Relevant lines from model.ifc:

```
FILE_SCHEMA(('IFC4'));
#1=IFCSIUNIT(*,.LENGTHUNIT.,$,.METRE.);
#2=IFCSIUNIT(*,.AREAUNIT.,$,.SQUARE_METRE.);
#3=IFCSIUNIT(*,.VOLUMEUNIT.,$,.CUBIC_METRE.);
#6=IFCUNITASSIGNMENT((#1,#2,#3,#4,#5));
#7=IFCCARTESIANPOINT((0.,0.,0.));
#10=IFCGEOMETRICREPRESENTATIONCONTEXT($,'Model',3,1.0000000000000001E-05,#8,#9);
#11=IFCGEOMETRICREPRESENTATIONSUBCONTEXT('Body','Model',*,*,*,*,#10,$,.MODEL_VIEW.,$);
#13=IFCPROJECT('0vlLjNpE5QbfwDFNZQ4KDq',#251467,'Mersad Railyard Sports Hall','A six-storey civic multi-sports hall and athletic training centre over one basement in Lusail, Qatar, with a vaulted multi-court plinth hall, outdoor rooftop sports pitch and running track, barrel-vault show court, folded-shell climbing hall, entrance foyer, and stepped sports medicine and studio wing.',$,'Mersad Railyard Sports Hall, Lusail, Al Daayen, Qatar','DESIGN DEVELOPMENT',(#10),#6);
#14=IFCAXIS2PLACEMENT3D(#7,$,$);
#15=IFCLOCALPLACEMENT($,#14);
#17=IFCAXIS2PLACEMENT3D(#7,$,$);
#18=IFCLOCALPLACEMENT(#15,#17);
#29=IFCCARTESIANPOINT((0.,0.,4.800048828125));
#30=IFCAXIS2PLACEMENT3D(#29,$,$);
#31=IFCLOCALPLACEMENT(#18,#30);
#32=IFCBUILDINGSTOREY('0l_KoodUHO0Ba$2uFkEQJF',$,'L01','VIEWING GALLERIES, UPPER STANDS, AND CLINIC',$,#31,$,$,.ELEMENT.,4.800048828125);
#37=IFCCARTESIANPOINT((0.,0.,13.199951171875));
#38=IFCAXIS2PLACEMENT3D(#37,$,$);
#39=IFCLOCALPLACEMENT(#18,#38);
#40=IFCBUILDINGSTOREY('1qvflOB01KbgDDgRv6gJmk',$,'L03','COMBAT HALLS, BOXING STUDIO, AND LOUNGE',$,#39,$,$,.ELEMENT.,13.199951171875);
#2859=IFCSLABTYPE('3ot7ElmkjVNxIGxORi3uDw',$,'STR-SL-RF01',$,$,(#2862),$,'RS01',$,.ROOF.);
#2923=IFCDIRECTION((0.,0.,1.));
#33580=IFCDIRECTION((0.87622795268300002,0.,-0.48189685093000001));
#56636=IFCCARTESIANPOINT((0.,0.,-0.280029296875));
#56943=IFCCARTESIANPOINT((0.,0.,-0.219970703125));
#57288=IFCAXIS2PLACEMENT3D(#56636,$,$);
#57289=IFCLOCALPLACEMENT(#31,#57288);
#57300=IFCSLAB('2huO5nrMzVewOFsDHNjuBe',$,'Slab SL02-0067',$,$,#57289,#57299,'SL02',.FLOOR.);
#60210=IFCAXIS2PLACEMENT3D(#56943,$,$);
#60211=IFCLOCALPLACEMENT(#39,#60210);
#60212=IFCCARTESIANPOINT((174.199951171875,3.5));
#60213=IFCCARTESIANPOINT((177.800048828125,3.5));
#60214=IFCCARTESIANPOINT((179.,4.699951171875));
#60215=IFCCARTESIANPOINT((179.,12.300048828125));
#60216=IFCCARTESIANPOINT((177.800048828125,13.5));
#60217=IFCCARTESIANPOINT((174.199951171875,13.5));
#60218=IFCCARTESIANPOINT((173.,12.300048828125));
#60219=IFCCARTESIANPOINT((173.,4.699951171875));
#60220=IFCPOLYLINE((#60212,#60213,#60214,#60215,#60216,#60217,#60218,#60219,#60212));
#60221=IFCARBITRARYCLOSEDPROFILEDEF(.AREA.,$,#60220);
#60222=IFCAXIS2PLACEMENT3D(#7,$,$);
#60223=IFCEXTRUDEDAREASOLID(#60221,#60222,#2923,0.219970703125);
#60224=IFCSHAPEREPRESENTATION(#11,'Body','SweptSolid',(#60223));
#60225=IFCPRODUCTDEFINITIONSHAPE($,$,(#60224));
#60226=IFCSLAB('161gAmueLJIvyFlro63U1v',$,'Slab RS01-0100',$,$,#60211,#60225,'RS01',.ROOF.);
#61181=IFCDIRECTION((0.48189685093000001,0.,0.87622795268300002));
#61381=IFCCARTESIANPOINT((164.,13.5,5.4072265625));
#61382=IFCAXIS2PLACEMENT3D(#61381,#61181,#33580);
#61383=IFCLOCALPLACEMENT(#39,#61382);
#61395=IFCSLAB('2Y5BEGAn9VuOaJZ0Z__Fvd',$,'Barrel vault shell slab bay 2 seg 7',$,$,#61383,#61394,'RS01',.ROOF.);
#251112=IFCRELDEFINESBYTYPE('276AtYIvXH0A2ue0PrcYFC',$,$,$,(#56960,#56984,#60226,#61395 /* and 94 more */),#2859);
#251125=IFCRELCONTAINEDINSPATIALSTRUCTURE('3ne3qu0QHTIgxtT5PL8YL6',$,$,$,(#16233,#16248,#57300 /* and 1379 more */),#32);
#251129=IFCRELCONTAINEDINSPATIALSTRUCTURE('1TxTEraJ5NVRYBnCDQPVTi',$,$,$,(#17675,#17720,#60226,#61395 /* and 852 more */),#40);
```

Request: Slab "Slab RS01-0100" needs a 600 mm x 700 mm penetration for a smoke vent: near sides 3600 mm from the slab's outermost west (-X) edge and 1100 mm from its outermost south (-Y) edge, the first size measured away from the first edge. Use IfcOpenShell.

```python
import numpy as np
import ifcopenshell
import ifcopenshell.api.feature
import ifcopenshell.api.geometry
import ifcopenshell.api.root
import ifcopenshell.geom
import ifcopenshell.util.placement
import ifcopenshell.util.representation
import ifcopenshell.util.shape
import ifcopenshell.util.unit

model = ifcopenshell.open("model.ifc")
unit_scale = ifcopenshell.util.unit.calculate_unit_scale(model)
settings = ifcopenshell.geom.settings()


def volume(element):
    """Net volume in cubic metres, openings subtracted."""
    shape = ifcopenshell.geom.create_shape(settings, element)
    return ifcopenshell.util.shape.get_volume(shape.geometry)


slab = model.by_guid("161gAmueLJIvyFlro63U1v")
before = volume(slab)

# Extent in the slab's own axes, in metres. The edges named are its -X and -Y sides.
slab_shape = ifcopenshell.geom.create_shape(settings, slab)
vertices = ifcopenshell.util.shape.get_vertices(slab_shape.geometry)
x_min, y_min, bottom = vertices.min(axis=0)
top = vertices[:, 2].max()

opening = ifcopenshell.api.root.create_entity(model, ifc_class="IfcOpeningElement", name="Smoke vent opening", predefined_type="OPENING")
context = ifcopenshell.util.representation.get_context(model, "Model", "Body", "MODEL_VIEW")
width, depth = 0.6, 0.7
outline = [(0.0, 0.0), (width, 0.0), (width, depth), (0.0, depth), (0.0, 0.0)]
# Overshoot both faces by 50 mm so the cut is clean.
shape = ifcopenshell.api.geometry.add_slab_representation(
    model, context=context, depth=top - bottom + 0.1, polyline=outline
)
ifcopenshell.api.geometry.assign_representation(model, product=opening, representation=shape)

matrix = ifcopenshell.util.placement.get_local_placement(slab.ObjectPlacement)
matrix[:, 3] = matrix @ np.append(np.array([x_min + 3.6, y_min + 1.1, bottom - 0.05]) / unit_scale, 1.0)
ifcopenshell.api.geometry.edit_object_placement(model, product=opening, matrix=matrix, is_si=False)
ifcopenshell.api.feature.add_feature(model, feature=opening, element=slab)

after = volume(slab)

print(f"slab volume {before:.3f} -> {after:.3f} m3")

model.write("model-out.ifc")
```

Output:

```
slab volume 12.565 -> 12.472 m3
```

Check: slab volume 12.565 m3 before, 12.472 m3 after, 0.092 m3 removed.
